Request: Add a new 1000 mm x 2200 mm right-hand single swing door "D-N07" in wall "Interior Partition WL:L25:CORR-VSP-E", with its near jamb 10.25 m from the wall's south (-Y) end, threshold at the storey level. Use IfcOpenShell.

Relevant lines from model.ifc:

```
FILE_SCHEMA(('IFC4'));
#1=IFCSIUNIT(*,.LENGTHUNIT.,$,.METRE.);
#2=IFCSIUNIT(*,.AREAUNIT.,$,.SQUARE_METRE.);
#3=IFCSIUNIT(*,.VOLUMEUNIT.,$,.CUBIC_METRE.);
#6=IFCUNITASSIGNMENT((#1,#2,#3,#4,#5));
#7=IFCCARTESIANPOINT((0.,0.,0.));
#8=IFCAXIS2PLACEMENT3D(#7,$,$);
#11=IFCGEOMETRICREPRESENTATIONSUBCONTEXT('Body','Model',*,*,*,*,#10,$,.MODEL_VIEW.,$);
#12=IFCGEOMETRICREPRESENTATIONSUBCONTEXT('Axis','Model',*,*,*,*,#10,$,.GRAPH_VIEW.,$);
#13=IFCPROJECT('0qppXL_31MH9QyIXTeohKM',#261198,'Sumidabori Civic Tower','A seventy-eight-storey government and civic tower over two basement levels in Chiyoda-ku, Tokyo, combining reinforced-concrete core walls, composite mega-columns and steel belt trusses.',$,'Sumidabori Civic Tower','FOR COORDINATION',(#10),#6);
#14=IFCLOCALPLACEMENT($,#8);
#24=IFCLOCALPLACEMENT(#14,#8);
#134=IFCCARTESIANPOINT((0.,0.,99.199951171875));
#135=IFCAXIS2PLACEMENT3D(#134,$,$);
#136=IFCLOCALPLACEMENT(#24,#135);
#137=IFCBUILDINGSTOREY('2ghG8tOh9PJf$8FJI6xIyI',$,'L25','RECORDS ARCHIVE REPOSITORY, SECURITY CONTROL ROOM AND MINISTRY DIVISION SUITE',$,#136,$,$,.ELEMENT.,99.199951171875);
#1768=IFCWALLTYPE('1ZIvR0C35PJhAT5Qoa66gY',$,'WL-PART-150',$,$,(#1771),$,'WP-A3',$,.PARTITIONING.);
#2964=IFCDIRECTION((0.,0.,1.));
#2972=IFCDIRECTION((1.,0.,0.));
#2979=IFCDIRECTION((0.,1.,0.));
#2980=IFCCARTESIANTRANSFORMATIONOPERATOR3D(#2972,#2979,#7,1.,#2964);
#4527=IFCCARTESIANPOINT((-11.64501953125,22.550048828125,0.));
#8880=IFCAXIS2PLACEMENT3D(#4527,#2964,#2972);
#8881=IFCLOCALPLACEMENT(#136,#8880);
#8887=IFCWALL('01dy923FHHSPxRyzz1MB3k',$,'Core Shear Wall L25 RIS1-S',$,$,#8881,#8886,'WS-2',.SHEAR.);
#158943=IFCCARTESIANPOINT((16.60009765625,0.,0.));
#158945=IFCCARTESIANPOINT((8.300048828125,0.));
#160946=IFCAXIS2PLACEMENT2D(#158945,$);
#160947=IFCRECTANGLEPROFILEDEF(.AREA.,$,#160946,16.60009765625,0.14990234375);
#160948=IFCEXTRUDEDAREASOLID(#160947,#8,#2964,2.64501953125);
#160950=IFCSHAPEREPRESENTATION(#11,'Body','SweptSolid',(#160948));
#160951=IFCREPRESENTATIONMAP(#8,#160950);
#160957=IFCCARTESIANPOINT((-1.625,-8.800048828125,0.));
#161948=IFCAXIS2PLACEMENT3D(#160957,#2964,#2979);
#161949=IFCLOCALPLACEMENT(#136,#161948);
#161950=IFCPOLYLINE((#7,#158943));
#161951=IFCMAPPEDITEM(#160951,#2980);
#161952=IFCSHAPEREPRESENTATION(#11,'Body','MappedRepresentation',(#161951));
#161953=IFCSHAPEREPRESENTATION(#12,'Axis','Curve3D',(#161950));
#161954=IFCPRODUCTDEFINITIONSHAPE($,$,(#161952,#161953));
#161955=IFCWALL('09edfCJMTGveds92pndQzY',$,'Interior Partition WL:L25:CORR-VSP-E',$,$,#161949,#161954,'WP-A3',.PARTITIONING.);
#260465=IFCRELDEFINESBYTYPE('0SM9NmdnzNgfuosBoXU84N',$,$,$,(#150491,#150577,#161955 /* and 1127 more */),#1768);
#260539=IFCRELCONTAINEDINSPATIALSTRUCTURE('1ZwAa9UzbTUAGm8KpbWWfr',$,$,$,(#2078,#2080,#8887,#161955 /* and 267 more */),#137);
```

```python
import numpy as np
import ifcopenshell
import ifcopenshell.api.feature
import ifcopenshell.api.geometry
import ifcopenshell.api.root
import ifcopenshell.api.spatial
import ifcopenshell.geom
import ifcopenshell.util.element
import ifcopenshell.util.placement
import ifcopenshell.util.representation
import ifcopenshell.util.shape
import ifcopenshell.util.unit

model = ifcopenshell.open("model.ifc")
unit_scale = ifcopenshell.util.unit.calculate_unit_scale(model)
settings = ifcopenshell.geom.settings()


def volume(element):
    """Net volume in cubic metres, openings subtracted."""
    shape = ifcopenshell.geom.create_shape(settings, element)
    return ifcopenshell.util.shape.get_volume(shape.geometry)


wall = model.by_id(161955)
storey = ifcopenshell.util.element.get_container(wall, ifc_class="IfcBuildingStorey")
context = ifcopenshell.util.representation.get_context(model, "Model", "Body", "MODEL_VIEW")
before = volume(wall)

width, height, from_end, sill = 1, 2.2, 10.25, 0.0  # metres

# The wall runs along its own X axis, and the end named is its -X end.
wall_shape = ifcopenshell.geom.create_shape(settings, wall)
x, y, z = ifcopenshell.util.shape.get_vertices(wall_shape.geometry).T
start = x.min() + from_end
face, thickness = float(y.min()), float(y.max() - y.min())
wall_matrix = ifcopenshell.util.placement.get_local_placement(wall.ObjectPlacement)
level = ifcopenshell.util.placement.get_local_placement(storey.ObjectPlacement)[2, 3]


def in_wall(x, y):
    """Placement at x, y metres in the wall's axes, at sill height."""
    matrix = wall_matrix.copy()
    matrix[:, 3] = wall_matrix @ np.array([x / unit_scale, y / unit_scale, 0.0, 1.0])
    matrix[2, 3] = level + sill / unit_scale
    return matrix


# Opening: a box that overshoots both wall faces by 50 mm.
opening = ifcopenshell.api.root.create_entity(model, ifc_class="IfcOpeningElement", predefined_type="OPENING")
box = ifcopenshell.api.geometry.add_wall_representation(
    model, context=context, length=width, height=height, thickness=thickness + 0.1
)
ifcopenshell.api.geometry.assign_representation(model, product=opening, representation=box)
ifcopenshell.api.geometry.edit_object_placement(model, product=opening, matrix=in_wall(start, face - 0.05), is_si=False)
ifcopenshell.api.feature.add_feature(model, feature=opening, element=wall)

door = ifcopenshell.api.root.create_entity(model, ifc_class="IfcDoor", name="D-N07", predefined_type="DOOR")
door.OverallWidth, door.OverallHeight = width / unit_scale, height / unit_scale
door.OperationType = "SINGLE_SWING_RIGHT"
body = ifcopenshell.api.geometry.add_door_representation(
    model,
    context=context,
    overall_width=door.OverallWidth,
    overall_height=door.OverallHeight,
    operation_type="SINGLE_SWING_RIGHT",
    lining_properties={"LiningDepth": thickness / unit_scale, "ThresholdDepth": thickness / unit_scale},
)
ifcopenshell.api.geometry.assign_representation(model, product=door, representation=body)
ifcopenshell.api.spatial.assign_container(model, products=[door], relating_structure=storey)
ifcopenshell.api.feature.add_filling(model, opening=opening, element=door)

# The lining spans the wall, so the door starts at the wall face.
ifcopenshell.api.geometry.edit_object_placement(model, product=door, matrix=in_wall(start, face), is_si=False)

after = volume(wall)

print(f"wall volume {before:.3f} -> {after:.3f} m3")

model.write("model-out.ifc")
```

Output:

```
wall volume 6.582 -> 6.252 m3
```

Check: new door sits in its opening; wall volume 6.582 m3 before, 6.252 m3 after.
